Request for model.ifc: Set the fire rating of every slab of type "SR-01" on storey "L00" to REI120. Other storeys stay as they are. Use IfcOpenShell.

First a look at what the model holds.

```python
import ifcopenshell
import ifcopenshell.util.element

model = ifcopenshell.open("model.ifc")
print(model.schema)
storey = next(s for s in model.by_type("IfcBuildingStorey") if s.Name == "L00")
slabs = [e for e in ifcopenshell.util.element.get_decomposition(storey) if e.is_a("IfcSlab")]
seen = {}
for e in slabs:
    element_type = ifcopenshell.util.element.get_type(e)
    key = (element_type.Name if element_type != e and element_type else None, ifcopenshell.util.element.get_pset(e, "Pset_SlabCommon", "FireRating"))
    seen[key] = seen.get(key, 0) + 1
for (name, value), count in sorted(seen.items(), key=str):
    print(count, "x", name, "|", value)
```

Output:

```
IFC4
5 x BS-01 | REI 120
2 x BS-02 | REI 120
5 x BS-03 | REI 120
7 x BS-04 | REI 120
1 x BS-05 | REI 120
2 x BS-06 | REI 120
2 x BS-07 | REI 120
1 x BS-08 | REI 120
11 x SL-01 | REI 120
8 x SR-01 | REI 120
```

```python
import ifcopenshell
import ifcopenshell.api.pset
import ifcopenshell.util.element

model = ifcopenshell.open("model.ifc")

storey = next(s for s in model.by_type("IfcBuildingStorey") if s.Name == "L00")
slabs = [e for e in ifcopenshell.util.element.get_decomposition(storey) if e.is_a("IfcSlab")]

count = 0
for e in slabs:
    element_type = ifcopenshell.util.element.get_type(e)
    if element_type in (None, e) or element_type.Name != "SR-01":
        continue
    # add_pset returns the element's existing set when there is one.
    pset = ifcopenshell.api.pset.add_pset(model, product=e, name="Pset_SlabCommon")
    ifcopenshell.api.pset.edit_pset(model, pset=pset, properties={"FireRating": "REI120"})
    count += 1

print(count, "slabs updated")

model.write("model-out.ifc")
```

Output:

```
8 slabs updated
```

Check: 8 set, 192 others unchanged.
